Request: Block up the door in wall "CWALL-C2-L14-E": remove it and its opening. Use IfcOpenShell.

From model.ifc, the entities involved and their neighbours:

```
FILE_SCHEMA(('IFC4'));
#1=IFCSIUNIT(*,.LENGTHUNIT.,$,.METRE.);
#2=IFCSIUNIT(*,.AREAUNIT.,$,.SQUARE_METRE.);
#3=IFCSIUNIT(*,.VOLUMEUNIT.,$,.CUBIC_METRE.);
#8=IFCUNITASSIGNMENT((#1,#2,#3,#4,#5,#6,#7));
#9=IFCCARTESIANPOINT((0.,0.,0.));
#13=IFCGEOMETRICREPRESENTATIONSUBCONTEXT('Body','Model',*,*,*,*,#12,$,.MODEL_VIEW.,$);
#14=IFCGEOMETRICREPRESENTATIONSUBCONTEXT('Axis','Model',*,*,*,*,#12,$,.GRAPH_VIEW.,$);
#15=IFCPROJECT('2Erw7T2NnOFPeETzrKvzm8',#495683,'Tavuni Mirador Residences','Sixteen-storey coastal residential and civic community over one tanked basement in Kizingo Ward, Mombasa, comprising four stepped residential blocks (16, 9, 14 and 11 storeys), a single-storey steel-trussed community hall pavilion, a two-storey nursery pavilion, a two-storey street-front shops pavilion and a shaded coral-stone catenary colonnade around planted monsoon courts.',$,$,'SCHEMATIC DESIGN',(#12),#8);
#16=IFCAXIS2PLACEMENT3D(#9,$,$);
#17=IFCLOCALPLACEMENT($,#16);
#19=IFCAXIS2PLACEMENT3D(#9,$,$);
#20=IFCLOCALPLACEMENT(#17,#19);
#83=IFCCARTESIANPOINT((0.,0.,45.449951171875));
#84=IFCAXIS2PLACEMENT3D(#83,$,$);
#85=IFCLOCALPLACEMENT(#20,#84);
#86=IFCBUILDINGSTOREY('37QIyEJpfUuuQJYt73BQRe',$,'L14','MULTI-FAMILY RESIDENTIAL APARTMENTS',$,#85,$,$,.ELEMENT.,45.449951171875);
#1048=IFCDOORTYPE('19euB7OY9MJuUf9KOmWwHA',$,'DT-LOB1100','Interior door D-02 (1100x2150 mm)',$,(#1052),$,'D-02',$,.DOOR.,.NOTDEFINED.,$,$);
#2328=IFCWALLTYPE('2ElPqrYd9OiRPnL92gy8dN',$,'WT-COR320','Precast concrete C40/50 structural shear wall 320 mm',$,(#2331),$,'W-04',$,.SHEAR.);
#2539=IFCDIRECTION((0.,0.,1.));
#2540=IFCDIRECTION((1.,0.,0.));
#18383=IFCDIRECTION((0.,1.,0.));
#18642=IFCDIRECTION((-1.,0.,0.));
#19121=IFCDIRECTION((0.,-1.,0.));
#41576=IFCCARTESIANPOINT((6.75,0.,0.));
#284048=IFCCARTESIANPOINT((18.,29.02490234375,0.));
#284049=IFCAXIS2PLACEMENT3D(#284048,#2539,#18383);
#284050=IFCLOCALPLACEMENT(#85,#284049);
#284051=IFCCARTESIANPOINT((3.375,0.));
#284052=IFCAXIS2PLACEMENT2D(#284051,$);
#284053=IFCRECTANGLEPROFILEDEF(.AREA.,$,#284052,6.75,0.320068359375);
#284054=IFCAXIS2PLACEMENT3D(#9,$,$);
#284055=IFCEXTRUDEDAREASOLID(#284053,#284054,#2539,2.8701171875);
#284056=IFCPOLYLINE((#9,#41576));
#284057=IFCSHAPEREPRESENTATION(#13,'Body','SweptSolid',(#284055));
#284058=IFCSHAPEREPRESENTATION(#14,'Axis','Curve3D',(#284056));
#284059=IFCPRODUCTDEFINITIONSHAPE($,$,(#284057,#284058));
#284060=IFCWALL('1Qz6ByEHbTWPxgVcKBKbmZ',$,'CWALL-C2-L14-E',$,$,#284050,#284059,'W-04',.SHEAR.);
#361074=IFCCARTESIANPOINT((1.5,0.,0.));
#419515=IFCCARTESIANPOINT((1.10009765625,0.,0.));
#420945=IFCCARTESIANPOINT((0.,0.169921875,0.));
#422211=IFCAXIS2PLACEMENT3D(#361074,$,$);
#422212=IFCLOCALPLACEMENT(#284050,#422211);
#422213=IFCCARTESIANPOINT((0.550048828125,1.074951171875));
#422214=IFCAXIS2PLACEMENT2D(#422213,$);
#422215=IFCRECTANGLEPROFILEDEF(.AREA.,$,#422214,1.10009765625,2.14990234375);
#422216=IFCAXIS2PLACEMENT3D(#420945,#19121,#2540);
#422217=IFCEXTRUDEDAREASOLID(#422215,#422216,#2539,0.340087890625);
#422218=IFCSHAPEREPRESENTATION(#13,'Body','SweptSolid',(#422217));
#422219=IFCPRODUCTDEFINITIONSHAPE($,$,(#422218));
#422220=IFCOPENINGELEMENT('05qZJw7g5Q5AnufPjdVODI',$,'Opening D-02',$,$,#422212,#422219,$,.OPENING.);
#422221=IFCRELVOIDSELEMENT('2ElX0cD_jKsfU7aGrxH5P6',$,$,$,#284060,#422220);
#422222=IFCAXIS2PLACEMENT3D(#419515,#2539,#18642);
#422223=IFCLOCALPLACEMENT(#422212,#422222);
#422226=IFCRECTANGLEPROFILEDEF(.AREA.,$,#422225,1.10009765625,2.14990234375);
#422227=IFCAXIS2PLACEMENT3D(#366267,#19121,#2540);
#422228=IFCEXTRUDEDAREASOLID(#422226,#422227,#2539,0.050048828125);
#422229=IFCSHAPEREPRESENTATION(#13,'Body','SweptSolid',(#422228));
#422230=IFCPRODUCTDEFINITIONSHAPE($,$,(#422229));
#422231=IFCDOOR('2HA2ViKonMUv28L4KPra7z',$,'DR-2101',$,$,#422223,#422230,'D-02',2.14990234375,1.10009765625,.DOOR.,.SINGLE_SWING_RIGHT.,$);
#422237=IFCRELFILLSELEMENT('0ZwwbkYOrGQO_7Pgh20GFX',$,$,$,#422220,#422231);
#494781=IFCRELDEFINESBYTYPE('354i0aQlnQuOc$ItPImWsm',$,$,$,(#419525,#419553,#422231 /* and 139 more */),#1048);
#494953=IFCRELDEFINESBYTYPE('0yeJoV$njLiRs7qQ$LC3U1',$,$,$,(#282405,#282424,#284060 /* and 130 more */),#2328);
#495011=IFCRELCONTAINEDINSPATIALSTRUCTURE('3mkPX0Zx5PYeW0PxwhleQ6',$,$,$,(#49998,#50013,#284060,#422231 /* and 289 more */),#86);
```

```python
import ifcopenshell
import ifcopenshell.api.feature
import ifcopenshell.api.root
import ifcopenshell.geom
import ifcopenshell.util.shape

model = ifcopenshell.open("model.ifc")
settings = ifcopenshell.geom.settings()


def volume(element):
    """Net volume in cubic metres, openings subtracted."""
    shape = ifcopenshell.geom.create_shape(settings, element)
    return ifcopenshell.util.shape.get_volume(shape.geometry)


door = model.by_id(422231)
opening = door.FillsVoids[0].RelatingOpeningElement
wall = opening.VoidsElements[0].RelatingBuildingElement
before = volume(wall)

ifcopenshell.api.root.remove_product(model, product=door)
ifcopenshell.api.feature.remove_feature(model, feature=opening)

after = volume(wall)

print(f"wall volume {before:.3f} -> {after:.3f} m3")

model.write("model-out.ifc")
```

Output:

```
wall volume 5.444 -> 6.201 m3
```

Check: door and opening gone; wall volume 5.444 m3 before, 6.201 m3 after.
